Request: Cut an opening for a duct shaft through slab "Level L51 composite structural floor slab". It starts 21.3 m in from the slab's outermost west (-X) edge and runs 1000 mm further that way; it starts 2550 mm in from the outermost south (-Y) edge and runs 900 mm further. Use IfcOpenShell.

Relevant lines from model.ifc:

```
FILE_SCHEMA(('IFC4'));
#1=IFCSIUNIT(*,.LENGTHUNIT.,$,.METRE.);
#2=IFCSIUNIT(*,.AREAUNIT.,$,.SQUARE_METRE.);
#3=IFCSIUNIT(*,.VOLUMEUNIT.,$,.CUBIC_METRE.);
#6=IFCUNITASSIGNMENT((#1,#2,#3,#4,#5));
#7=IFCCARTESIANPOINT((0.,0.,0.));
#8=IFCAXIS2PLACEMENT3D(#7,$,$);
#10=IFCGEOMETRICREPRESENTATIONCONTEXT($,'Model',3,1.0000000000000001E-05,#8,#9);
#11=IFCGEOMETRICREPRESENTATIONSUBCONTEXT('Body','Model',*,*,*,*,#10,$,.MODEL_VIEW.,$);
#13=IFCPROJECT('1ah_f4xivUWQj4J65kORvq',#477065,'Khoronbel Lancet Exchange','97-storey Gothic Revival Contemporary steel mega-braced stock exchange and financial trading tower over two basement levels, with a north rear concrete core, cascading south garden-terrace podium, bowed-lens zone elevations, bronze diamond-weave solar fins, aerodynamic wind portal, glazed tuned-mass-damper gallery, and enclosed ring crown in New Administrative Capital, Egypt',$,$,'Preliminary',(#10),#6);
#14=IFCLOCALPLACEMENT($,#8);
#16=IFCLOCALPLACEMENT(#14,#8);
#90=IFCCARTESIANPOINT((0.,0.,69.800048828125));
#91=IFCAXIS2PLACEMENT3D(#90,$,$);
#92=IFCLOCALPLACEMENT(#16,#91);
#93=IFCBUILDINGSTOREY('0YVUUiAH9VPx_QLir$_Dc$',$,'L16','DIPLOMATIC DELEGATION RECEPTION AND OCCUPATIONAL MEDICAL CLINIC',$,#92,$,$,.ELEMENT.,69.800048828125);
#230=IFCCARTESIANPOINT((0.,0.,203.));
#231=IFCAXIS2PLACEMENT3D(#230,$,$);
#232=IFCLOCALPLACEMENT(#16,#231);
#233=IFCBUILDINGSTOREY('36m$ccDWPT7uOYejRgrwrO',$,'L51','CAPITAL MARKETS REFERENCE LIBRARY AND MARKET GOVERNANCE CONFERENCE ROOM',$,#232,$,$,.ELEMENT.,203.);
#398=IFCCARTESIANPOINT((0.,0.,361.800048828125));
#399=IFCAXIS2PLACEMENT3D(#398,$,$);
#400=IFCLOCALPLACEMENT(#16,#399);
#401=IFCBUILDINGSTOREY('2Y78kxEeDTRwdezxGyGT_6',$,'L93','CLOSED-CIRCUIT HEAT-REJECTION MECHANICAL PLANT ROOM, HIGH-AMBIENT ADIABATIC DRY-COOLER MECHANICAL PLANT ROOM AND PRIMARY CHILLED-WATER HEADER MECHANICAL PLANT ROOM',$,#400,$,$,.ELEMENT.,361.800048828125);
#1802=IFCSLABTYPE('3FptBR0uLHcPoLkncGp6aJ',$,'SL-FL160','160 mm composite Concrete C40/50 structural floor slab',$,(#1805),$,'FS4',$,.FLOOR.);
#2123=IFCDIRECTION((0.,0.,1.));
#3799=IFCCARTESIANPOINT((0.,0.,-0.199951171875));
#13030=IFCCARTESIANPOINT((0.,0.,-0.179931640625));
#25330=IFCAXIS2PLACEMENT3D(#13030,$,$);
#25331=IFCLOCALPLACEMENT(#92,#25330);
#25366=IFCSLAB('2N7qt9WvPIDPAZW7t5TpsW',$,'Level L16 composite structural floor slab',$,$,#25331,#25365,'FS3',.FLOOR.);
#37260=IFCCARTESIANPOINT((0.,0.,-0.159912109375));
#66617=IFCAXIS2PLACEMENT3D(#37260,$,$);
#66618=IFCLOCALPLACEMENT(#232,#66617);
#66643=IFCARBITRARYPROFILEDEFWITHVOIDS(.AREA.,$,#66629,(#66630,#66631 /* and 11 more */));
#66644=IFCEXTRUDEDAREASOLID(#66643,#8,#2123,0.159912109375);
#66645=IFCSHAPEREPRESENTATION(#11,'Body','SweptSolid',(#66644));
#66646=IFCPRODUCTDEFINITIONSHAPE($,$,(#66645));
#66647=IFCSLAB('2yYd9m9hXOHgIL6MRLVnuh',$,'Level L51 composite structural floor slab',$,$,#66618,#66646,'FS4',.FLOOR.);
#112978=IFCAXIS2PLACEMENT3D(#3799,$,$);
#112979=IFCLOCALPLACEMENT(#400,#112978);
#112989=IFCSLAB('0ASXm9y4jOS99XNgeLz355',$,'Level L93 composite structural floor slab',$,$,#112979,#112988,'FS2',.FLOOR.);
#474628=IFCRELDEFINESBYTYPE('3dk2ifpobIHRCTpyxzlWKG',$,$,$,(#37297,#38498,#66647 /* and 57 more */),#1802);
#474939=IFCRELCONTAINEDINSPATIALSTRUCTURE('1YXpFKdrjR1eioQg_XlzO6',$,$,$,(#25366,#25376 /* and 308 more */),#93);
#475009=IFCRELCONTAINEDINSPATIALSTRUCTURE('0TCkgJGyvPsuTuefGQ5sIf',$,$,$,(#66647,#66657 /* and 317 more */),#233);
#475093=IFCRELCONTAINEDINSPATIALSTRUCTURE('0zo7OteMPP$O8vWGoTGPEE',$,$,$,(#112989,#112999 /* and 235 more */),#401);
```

```python
import numpy as np
import ifcopenshell
import ifcopenshell.api.feature
import ifcopenshell.api.geometry
import ifcopenshell.api.root
import ifcopenshell.geom
import ifcopenshell.util.placement
import ifcopenshell.util.representation
import ifcopenshell.util.shape
import ifcopenshell.util.unit

model = ifcopenshell.open("model.ifc")
unit_scale = ifcopenshell.util.unit.calculate_unit_scale(model)
settings = ifcopenshell.geom.settings()


def volume(element):
    """Net volume in cubic metres, openings subtracted."""
    shape = ifcopenshell.geom.create_shape(settings, element)
    return ifcopenshell.util.shape.get_volume(shape.geometry)


slab = model.by_id(66647)
before = volume(slab)

# Extent in the slab's own axes, in metres. The edges named are its -X and -Y sides.
slab_shape = ifcopenshell.geom.create_shape(settings, slab)
vertices = ifcopenshell.util.shape.get_vertices(slab_shape.geometry)
x_min, y_min, bottom = vertices.min(axis=0)
top = vertices[:, 2].max()

opening = ifcopenshell.api.root.create_entity(model, ifc_class="IfcOpeningElement", name="Duct shaft opening", predefined_type="OPENING")
context = ifcopenshell.util.representation.get_context(model, "Model", "Body", "MODEL_VIEW")
width, depth = 1, 0.9
outline = [(0.0, 0.0), (width, 0.0), (width, depth), (0.0, depth), (0.0, 0.0)]
# Overshoot both faces by 50 mm so the cut is clean.
shape = ifcopenshell.api.geometry.add_slab_representation(
    model, context=context, depth=top - bottom + 0.1, polyline=outline
)
ifcopenshell.api.geometry.assign_representation(model, product=opening, representation=shape)

matrix = ifcopenshell.util.placement.get_local_placement(slab.ObjectPlacement)
matrix[:, 3] = matrix @ np.append(np.array([x_min + 21.3, y_min + 2.55, bottom - 0.05]) / unit_scale, 1.0)
ifcopenshell.api.geometry.edit_object_placement(model, product=opening, matrix=matrix, is_si=False)
ifcopenshell.api.feature.add_feature(model, feature=opening, element=slab)

after = volume(slab)

print(f"slab volume {before:.3f} -> {after:.3f} m3")

model.write("model-out.ifc")
```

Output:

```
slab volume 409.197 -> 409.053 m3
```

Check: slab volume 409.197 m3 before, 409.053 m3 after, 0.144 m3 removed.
